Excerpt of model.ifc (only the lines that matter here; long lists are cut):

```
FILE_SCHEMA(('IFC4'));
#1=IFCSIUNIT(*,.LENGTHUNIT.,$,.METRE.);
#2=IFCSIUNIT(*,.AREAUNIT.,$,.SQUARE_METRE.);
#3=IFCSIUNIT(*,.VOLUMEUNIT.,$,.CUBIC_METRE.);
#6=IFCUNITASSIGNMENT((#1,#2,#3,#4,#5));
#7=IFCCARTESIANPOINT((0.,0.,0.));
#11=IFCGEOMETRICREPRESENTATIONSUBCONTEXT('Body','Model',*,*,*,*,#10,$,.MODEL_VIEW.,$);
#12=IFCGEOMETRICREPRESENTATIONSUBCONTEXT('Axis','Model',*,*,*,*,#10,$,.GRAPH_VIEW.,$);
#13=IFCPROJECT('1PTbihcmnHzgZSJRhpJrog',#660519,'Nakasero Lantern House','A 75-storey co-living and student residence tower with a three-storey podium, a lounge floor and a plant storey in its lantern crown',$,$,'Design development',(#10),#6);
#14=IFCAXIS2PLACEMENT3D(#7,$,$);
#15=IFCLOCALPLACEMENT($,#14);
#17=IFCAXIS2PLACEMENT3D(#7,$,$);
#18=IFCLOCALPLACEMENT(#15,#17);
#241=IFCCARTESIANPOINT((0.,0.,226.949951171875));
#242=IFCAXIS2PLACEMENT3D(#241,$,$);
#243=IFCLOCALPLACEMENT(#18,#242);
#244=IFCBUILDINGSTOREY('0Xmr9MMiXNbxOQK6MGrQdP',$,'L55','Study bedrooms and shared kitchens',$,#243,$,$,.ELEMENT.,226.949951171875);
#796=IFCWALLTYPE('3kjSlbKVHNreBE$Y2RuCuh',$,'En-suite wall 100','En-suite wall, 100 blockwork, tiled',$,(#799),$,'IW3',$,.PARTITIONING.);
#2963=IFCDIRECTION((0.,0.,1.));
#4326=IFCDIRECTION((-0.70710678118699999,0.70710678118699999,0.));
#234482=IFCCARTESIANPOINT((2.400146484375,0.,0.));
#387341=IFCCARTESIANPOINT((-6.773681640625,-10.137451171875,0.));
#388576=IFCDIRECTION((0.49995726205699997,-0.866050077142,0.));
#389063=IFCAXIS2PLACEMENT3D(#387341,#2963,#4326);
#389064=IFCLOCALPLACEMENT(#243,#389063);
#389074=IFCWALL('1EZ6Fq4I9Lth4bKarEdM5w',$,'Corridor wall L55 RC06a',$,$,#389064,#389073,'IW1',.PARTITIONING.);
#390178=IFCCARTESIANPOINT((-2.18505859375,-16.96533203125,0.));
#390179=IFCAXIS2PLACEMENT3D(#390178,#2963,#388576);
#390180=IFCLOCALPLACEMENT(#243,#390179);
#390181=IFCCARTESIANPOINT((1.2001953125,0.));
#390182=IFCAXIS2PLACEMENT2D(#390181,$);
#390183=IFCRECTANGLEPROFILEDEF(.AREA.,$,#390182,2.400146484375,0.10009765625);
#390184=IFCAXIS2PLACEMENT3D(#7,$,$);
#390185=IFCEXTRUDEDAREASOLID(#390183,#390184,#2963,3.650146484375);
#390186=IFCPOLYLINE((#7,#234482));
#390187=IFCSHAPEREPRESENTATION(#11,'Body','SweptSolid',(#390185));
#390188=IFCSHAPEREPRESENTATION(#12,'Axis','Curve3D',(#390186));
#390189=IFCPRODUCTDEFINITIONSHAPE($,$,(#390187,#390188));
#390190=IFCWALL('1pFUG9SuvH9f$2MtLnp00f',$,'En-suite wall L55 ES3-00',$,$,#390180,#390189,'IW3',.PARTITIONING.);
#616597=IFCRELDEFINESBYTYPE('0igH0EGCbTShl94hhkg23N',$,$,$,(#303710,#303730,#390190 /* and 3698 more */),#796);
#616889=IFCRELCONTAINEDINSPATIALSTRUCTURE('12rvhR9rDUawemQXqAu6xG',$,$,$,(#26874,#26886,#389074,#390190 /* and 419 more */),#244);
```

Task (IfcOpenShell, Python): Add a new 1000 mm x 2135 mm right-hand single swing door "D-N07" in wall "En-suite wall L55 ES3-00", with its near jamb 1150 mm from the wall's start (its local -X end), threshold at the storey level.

```python
import numpy as np
import ifcopenshell
import ifcopenshell.api.feature
import ifcopenshell.api.geometry
import ifcopenshell.api.root
import ifcopenshell.api.spatial
import ifcopenshell.geom
import ifcopenshell.util.element
import ifcopenshell.util.placement
import ifcopenshell.util.representation
import ifcopenshell.util.shape
import ifcopenshell.util.unit

model = ifcopenshell.open("model.ifc")
unit_scale = ifcopenshell.util.unit.calculate_unit_scale(model)
settings = ifcopenshell.geom.settings()


def volume(element):
    """Net volume in cubic metres, openings subtracted."""
    shape = ifcopenshell.geom.create_shape(settings, element)
    return ifcopenshell.util.shape.get_volume(shape.geometry)


wall = model.by_id(390190)
storey = ifcopenshell.util.element.get_container(wall, ifc_class="IfcBuildingStorey")
context = ifcopenshell.util.representation.get_context(model, "Model", "Body", "MODEL_VIEW")
before = volume(wall)

width, height, from_end, sill = 1, 2.135, 1.15, 0.0  # metres

# The wall runs along its own X axis, and the end named is its -X end.
wall_shape = ifcopenshell.geom.create_shape(settings, wall)
x, y, z = ifcopenshell.util.shape.get_vertices(wall_shape.geometry).T
start = x.min() + from_end
face, thickness = float(y.min()), float(y.max() - y.min())
wall_matrix = ifcopenshell.util.placement.get_local_placement(wall.ObjectPlacement)
level = ifcopenshell.util.placement.get_local_placement(storey.ObjectPlacement)[2, 3]


def in_wall(x, y):
    """Placement at x, y metres in the wall's axes, at sill height."""
    matrix = wall_matrix.copy()
    matrix[:, 3] = wall_matrix @ np.array([x / unit_scale, y / unit_scale, 0.0, 1.0])
    matrix[2, 3] = level + sill / unit_scale
    return matrix


# Opening: a box that overshoots both wall faces by 50 mm.
opening = ifcopenshell.api.root.create_entity(model, ifc_class="IfcOpeningElement", predefined_type="OPENING")
box = ifcopenshell.api.geometry.add_wall_representation(
    model, context=context, length=width, height=height, thickness=thickness + 0.1
)
ifcopenshell.api.geometry.assign_representation(model, product=opening, representation=box)
ifcopenshell.api.geometry.edit_object_placement(model, product=opening, matrix=in_wall(start, face - 0.05), is_si=False)
ifcopenshell.api.feature.add_feature(model, feature=opening, element=wall)

door = ifcopenshell.api.root.create_entity(model, ifc_class="IfcDoor", name="D-N07", predefined_type="DOOR")
door.OverallWidth, door.OverallHeight = width / unit_scale, height / unit_scale
door.OperationType = "SINGLE_SWING_RIGHT"
body = ifcopenshell.api.geometry.add_door_representation(
    model,
    context=context,
    overall_width=door.OverallWidth,
    overall_height=door.OverallHeight,
    operation_type="SINGLE_SWING_RIGHT",
    lining_properties={"LiningDepth": thickness / unit_scale, "ThresholdDepth": thickness / unit_scale},
)
ifcopenshell.api.geometry.assign_representation(model, product=door, representation=body)
ifcopenshell.api.spatial.assign_container(model, products=[door], relating_structure=storey)
ifcopenshell.api.feature.add_filling(model, opening=opening, element=door)

# The lining spans the wall, so the door starts at the wall face.
ifcopenshell.api.geometry.edit_object_placement(model, product=door, matrix=in_wall(start, face), is_si=False)

after = volume(wall)

print(f"wall volume {before:.3f} -> {after:.3f} m3")

model.write("model_v2.ifc")
```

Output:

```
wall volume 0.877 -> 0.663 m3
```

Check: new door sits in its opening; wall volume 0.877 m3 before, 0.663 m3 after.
